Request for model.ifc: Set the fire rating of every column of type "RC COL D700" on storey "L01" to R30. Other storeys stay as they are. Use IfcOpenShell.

First a look at what the model holds.

```python
import ifcopenshell
import ifcopenshell.util.element

model = ifcopenshell.open("model.ifc")
print(model.schema)
storey = next(s for s in model.by_type("IfcBuildingStorey") if s.Name == "L01")
columns = [e for e in ifcopenshell.util.element.get_decomposition(storey) if e.is_a("IfcColumn")]
seen = {}
for e in columns:
    element_type = ifcopenshell.util.element.get_type(e)
    key = (element_type.Name if element_type != e and element_type else None, ifcopenshell.util.element.get_pset(e, "Pset_ColumnCommon", "FireRating"))
    seen[key] = seen.get(key, 0) + 1
for (name, value), count in sorted(seen.items(), key=str):
    print(count, "x", name, "|", value)
```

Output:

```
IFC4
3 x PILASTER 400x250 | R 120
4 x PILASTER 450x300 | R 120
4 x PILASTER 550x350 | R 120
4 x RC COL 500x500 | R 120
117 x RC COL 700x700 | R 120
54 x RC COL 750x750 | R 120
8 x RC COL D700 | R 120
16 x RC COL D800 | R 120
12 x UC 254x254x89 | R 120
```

```python
import ifcopenshell
import ifcopenshell.api.pset
import ifcopenshell.util.element

model = ifcopenshell.open("model.ifc")

storey = next(s for s in model.by_type("IfcBuildingStorey") if s.Name == "L01")
columns = [e for e in ifcopenshell.util.element.get_decomposition(storey) if e.is_a("IfcColumn")]

count = 0
for e in columns:
    element_type = ifcopenshell.util.element.get_type(e)
    if element_type in (None, e) or element_type.Name != "RC COL D700":
        continue
    # add_pset returns the element's existing set when there is one.
    pset = ifcopenshell.api.pset.add_pset(model, product=e, name="Pset_ColumnCommon")
    ifcopenshell.api.pset.edit_pset(model, pset=pset, properties={"FireRating": "R30"})
    count += 1

print(count, "columns updated")

model.write("model_v2.ifc")
```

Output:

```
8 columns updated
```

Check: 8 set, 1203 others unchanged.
